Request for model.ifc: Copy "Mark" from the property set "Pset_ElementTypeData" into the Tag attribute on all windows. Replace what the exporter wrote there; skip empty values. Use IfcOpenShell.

First a look at what the model holds.

```python
import ifcopenshell
import ifcopenshell.util.element

model = ifcopenshell.open("model.ifc")
print(model.schema)
windows = model.by_type("IfcWindow")
print(len(windows), "windows")
for e in windows[:8]:
    source = ifcopenshell.util.element.get_pset(e, "Pset_ElementTypeData", "Mark")
    target = e.Tag
    print(e.id(), repr(source), repr(target), sep=" | ")
```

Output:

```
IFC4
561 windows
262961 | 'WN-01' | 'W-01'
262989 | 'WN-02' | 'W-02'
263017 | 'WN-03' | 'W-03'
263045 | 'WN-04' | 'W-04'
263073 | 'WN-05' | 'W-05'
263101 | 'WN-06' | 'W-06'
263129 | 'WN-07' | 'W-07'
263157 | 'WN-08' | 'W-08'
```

```python
import ifcopenshell
import ifcopenshell.util.element

model = ifcopenshell.open("model.ifc")

count = 0
for e in model.by_type("IfcWindow"):
    value = ifcopenshell.util.element.get_pset(e, "Pset_ElementTypeData", "Mark")
    current = e.Tag
    if not value or not value.strip() or current == value:
        continue
    e.Tag = value
    count += 1

print(count, "windows updated")

model.write("model-out.ifc")
```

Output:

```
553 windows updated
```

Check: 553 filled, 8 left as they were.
